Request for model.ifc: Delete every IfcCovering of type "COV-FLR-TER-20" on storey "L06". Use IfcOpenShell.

First a look at what the model holds.

```python
import ifcopenshell
import ifcopenshell.util.element

model = ifcopenshell.open("model.ifc")
print(model.schema)
storey = next(s for s in model.by_type("IfcBuildingStorey") if s.Name == "L06")
coverings = [e for e in ifcopenshell.util.element.get_decomposition(storey) if e.is_a("IfcCovering")]
seen = {}
for e in coverings:
    element_type = ifcopenshell.util.element.get_type(e)
    name = element_type.Name if element_type not in (None, e) else None
    seen[name] = seen.get(name, 0) + 1
for name, count in sorted(seen.items(), key=str):
    print(count, "x", name)
```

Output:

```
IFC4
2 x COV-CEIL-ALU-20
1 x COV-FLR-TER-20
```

```python
import ifcopenshell
import ifcopenshell.api.root
import ifcopenshell.util.element

model = ifcopenshell.open("model.ifc")

storey = next(s for s in model.by_type("IfcBuildingStorey") if s.Name == "L06")
coverings = [e for e in ifcopenshell.util.element.get_decomposition(storey) if e.is_a("IfcCovering")]
targets = [e for e in coverings if (t := ifcopenshell.util.element.get_type(e)) not in (None, e) and t.Name == "COV-FLR-TER-20"]

for e in targets:
    ifcopenshell.api.root.remove_product(model, product=e)
print(len(targets), "removed")

model.write("model_updated.ifc")
```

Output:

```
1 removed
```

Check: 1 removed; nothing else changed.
